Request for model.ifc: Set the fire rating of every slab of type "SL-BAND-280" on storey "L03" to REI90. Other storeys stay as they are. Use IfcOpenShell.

First a look at what the model holds.

```python
import ifcopenshell
import ifcopenshell.util.element

model = ifcopenshell.open("model.ifc")
print(model.schema)
storey = next(s for s in model.by_type("IfcBuildingStorey") if s.Name == "L03")
slabs = [e for e in ifcopenshell.util.element.get_decomposition(storey) if e.is_a("IfcSlab")]
seen = {}
for e in slabs:
    element_type = ifcopenshell.util.element.get_type(e)
    key = (element_type.Name if element_type != e and element_type else None, ifcopenshell.util.element.get_pset(e, "Pset_SlabCommon", "FireRating"))
    seen[key] = seen.get(key, 0) + 1
for (name, value), count in sorted(seen.items(), key=str):
    print(count, "x", name, "|", value)
```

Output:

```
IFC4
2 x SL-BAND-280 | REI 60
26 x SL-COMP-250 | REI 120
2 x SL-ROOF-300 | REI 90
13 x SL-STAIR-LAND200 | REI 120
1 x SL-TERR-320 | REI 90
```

```python
import ifcopenshell
import ifcopenshell.api.pset
import ifcopenshell.util.element

model = ifcopenshell.open("model.ifc")

storey = next(s for s in model.by_type("IfcBuildingStorey") if s.Name == "L03")
slabs = [e for e in ifcopenshell.util.element.get_decomposition(storey) if e.is_a("IfcSlab")]

count = 0
for e in slabs:
    element_type = ifcopenshell.util.element.get_type(e)
    if element_type in (None, e) or element_type.Name != "SL-BAND-280":
        continue
    # add_pset returns the element's existing set when there is one.
    pset = ifcopenshell.api.pset.add_pset(model, product=e, name="Pset_SlabCommon")
    ifcopenshell.api.pset.edit_pset(model, pset=pset, properties={"FireRating": "REI90"})
    count += 1

print(count, "slabs updated")

model.write("model-out.ifc")
```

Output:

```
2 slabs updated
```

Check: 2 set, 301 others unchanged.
